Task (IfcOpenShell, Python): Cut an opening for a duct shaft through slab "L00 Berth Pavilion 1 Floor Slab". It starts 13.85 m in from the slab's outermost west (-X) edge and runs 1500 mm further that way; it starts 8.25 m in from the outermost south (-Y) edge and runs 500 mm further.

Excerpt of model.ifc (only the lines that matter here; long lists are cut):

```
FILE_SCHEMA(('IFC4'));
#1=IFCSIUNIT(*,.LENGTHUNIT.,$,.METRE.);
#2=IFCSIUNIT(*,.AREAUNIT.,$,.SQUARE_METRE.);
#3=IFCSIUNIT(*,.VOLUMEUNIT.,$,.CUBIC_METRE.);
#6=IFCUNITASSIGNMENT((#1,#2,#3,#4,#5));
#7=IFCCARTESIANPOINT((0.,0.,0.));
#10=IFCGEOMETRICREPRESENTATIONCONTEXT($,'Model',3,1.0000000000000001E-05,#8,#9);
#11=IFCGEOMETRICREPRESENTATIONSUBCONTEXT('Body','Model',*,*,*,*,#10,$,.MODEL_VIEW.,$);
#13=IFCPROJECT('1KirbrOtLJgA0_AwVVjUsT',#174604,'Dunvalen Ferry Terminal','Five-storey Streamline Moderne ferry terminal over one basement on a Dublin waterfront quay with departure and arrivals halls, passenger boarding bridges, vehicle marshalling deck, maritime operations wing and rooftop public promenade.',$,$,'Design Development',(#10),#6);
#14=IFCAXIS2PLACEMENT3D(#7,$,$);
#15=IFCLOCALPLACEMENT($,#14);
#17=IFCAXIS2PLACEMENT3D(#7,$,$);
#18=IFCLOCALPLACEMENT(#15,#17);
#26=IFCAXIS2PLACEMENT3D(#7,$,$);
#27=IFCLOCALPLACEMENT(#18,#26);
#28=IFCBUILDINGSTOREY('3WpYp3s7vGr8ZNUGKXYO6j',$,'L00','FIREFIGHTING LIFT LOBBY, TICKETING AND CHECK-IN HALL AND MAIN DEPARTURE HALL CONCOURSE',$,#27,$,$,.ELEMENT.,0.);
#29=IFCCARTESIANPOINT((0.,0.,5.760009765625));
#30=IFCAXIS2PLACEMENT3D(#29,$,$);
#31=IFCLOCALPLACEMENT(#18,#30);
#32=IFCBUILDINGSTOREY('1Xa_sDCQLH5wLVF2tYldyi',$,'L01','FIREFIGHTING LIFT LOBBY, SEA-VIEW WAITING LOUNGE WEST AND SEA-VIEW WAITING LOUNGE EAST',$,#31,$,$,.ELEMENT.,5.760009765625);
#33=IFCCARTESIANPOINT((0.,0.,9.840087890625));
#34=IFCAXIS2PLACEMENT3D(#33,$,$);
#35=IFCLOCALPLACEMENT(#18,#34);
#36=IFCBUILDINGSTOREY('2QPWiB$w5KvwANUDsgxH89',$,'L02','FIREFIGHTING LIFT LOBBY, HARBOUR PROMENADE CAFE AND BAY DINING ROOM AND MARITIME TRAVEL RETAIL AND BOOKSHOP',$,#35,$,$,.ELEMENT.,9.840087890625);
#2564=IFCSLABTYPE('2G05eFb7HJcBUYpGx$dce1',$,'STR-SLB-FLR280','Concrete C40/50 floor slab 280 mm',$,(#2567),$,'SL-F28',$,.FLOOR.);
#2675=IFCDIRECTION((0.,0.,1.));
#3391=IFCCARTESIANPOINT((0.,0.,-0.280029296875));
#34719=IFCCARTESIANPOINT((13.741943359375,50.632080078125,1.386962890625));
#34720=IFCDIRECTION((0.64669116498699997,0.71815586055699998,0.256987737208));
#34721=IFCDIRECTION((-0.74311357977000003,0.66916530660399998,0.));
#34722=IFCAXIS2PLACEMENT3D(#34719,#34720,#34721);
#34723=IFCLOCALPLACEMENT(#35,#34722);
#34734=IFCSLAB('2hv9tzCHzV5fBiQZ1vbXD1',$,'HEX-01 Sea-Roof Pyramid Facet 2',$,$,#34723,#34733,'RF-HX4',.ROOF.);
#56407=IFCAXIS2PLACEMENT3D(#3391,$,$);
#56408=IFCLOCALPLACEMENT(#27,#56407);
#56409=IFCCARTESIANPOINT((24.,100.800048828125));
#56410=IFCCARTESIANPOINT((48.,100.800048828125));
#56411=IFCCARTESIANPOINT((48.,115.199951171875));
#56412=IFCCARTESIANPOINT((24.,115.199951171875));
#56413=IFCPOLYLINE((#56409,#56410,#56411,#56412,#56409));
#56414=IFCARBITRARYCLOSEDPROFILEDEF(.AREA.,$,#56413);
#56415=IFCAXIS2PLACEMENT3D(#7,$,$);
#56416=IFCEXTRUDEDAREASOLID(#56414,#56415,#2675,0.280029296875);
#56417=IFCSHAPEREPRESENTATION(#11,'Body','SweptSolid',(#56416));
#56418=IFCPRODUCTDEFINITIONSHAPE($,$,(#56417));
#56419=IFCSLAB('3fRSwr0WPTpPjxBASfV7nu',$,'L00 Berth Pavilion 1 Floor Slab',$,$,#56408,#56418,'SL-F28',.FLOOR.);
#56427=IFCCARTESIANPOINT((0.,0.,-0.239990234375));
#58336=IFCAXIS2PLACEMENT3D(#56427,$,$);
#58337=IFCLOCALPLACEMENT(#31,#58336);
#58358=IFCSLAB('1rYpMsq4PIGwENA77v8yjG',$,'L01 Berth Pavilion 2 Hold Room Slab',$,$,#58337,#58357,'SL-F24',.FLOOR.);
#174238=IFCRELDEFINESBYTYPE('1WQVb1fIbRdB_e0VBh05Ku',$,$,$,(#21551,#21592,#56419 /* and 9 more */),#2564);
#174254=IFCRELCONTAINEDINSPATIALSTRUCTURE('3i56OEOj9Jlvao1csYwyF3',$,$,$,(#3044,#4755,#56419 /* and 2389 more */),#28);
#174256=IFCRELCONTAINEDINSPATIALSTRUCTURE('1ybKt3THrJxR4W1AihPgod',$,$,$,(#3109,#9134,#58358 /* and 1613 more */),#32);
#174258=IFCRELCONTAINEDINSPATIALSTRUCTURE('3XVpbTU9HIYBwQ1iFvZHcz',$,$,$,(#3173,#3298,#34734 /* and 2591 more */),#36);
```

```python
import numpy as np
import ifcopenshell
import ifcopenshell.api.feature
import ifcopenshell.api.geometry
import ifcopenshell.api.root
import ifcopenshell.geom
import ifcopenshell.util.placement
import ifcopenshell.util.representation
import ifcopenshell.util.shape
import ifcopenshell.util.unit

model = ifcopenshell.open("model.ifc")
unit_scale = ifcopenshell.util.unit.calculate_unit_scale(model)
settings = ifcopenshell.geom.settings()


def volume(element):
    """Net volume in cubic metres, openings subtracted."""
    shape = ifcopenshell.geom.create_shape(settings, element)
    return ifcopenshell.util.shape.get_volume(shape.geometry)


slab = model.by_id(56419)
before = volume(slab)

# Extent in the slab's own axes, in metres. The edges named are its -X and -Y sides.
slab_shape = ifcopenshell.geom.create_shape(settings, slab)
vertices = ifcopenshell.util.shape.get_vertices(slab_shape.geometry)
x_min, y_min, bottom = vertices.min(axis=0)
top = vertices[:, 2].max()

opening = ifcopenshell.api.root.create_entity(model, ifc_class="IfcOpeningElement", name="Duct shaft opening", predefined_type="OPENING")
context = ifcopenshell.util.representation.get_context(model, "Model", "Body", "MODEL_VIEW")
width, depth = 1.5, 0.5
outline = [(0.0, 0.0), (width, 0.0), (width, depth), (0.0, depth), (0.0, 0.0)]
# Overshoot both faces by 50 mm so the cut is clean.
shape = ifcopenshell.api.geometry.add_slab_representation(
    model, context=context, depth=top - bottom + 0.1, polyline=outline
)
ifcopenshell.api.geometry.assign_representation(model, product=opening, representation=shape)

matrix = ifcopenshell.util.placement.get_local_placement(slab.ObjectPlacement)
matrix[:, 3] = matrix @ np.append(np.array([x_min + 13.85, y_min + 8.25, bottom - 0.05]) / unit_scale, 1.0)
ifcopenshell.api.geometry.edit_object_placement(model, product=opening, matrix=matrix, is_si=False)
ifcopenshell.api.feature.add_feature(model, feature=opening, element=slab)

after = volume(slab)

print(f"slab volume {before:.3f} -> {after:.3f} m3")

model.write("model-out.ifc")
```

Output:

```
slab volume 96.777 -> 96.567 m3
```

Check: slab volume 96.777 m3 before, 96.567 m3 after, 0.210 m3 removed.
